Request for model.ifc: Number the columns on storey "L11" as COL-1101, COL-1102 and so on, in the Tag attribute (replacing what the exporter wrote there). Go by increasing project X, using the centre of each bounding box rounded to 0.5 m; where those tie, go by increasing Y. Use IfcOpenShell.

First a look at what the model holds.

```python
import ifcopenshell
import ifcopenshell.util.element
import ifcopenshell.util.placement

model = ifcopenshell.open("model.ifc")
print(model.schema)
storey = next(s for s in model.by_type("IfcBuildingStorey") if s.Name == "L11")
columns = [e for e in ifcopenshell.util.element.get_decomposition(storey) if e.is_a("IfcColumn")]
for e in sorted(columns, key=lambda e: e.id()):
    origin = ifcopenshell.util.placement.get_local_placement(e.ObjectPlacement)[:3, 3]
    print(e.id(), e.Tag, e.Name, origin.round(2) + 0.0, sep=" | ")
```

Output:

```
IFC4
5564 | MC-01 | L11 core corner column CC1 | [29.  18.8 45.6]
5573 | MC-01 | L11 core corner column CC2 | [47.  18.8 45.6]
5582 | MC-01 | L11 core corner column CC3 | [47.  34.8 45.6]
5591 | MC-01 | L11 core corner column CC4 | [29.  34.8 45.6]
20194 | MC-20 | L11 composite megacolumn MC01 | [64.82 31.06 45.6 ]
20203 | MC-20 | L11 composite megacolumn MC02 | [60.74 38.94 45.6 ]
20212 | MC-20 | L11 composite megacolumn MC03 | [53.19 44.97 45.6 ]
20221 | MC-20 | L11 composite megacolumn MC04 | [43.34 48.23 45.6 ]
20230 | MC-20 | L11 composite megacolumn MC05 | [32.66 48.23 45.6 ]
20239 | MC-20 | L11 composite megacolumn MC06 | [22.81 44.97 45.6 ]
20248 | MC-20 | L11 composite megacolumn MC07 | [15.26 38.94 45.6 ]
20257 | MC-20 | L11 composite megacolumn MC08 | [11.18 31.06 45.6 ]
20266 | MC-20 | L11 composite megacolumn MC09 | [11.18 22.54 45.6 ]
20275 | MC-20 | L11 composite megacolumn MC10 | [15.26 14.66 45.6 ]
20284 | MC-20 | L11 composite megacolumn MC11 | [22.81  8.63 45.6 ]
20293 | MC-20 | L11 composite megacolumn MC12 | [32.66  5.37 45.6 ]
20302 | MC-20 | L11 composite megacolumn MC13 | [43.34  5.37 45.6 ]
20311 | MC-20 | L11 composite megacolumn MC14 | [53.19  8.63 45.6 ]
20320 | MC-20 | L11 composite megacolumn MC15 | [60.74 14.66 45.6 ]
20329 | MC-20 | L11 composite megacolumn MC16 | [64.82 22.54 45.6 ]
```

```python
import ifcopenshell
import ifcopenshell.geom
import ifcopenshell.util.element
import ifcopenshell.util.shape

model = ifcopenshell.open("model.ifc")
settings = ifcopenshell.geom.settings()
settings.set("use-world-coords", True)


def centre(element):
    shape = ifcopenshell.geom.create_shape(settings, element)
    return ifcopenshell.util.shape.get_bbox_centroid(shape.geometry)


storey = next(s for s in model.by_type("IfcBuildingStorey") if s.Name == "L11")
columns = [e for e in ifcopenshell.util.element.get_decomposition(storey) if e.is_a("IfcColumn")]

# Insertion points can sit at a corner or the storey origin, so sort by the geometry (in metres).
centres = {e: centre(e) for e in columns}
columns.sort(key=lambda e: (round(centres[e][0] / 0.5), centres[e][1]))

for i, e in enumerate(columns, start=1):
    number = f"COL-11{i:02d}"
    e.Tag = number
    print(e.id(), number)

model.write("model_rev.ifc")
```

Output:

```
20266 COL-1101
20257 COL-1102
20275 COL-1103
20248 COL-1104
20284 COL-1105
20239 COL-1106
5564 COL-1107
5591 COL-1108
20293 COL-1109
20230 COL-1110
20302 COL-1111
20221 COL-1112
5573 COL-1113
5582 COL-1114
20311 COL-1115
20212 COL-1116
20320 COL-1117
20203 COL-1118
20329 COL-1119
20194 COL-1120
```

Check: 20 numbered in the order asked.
